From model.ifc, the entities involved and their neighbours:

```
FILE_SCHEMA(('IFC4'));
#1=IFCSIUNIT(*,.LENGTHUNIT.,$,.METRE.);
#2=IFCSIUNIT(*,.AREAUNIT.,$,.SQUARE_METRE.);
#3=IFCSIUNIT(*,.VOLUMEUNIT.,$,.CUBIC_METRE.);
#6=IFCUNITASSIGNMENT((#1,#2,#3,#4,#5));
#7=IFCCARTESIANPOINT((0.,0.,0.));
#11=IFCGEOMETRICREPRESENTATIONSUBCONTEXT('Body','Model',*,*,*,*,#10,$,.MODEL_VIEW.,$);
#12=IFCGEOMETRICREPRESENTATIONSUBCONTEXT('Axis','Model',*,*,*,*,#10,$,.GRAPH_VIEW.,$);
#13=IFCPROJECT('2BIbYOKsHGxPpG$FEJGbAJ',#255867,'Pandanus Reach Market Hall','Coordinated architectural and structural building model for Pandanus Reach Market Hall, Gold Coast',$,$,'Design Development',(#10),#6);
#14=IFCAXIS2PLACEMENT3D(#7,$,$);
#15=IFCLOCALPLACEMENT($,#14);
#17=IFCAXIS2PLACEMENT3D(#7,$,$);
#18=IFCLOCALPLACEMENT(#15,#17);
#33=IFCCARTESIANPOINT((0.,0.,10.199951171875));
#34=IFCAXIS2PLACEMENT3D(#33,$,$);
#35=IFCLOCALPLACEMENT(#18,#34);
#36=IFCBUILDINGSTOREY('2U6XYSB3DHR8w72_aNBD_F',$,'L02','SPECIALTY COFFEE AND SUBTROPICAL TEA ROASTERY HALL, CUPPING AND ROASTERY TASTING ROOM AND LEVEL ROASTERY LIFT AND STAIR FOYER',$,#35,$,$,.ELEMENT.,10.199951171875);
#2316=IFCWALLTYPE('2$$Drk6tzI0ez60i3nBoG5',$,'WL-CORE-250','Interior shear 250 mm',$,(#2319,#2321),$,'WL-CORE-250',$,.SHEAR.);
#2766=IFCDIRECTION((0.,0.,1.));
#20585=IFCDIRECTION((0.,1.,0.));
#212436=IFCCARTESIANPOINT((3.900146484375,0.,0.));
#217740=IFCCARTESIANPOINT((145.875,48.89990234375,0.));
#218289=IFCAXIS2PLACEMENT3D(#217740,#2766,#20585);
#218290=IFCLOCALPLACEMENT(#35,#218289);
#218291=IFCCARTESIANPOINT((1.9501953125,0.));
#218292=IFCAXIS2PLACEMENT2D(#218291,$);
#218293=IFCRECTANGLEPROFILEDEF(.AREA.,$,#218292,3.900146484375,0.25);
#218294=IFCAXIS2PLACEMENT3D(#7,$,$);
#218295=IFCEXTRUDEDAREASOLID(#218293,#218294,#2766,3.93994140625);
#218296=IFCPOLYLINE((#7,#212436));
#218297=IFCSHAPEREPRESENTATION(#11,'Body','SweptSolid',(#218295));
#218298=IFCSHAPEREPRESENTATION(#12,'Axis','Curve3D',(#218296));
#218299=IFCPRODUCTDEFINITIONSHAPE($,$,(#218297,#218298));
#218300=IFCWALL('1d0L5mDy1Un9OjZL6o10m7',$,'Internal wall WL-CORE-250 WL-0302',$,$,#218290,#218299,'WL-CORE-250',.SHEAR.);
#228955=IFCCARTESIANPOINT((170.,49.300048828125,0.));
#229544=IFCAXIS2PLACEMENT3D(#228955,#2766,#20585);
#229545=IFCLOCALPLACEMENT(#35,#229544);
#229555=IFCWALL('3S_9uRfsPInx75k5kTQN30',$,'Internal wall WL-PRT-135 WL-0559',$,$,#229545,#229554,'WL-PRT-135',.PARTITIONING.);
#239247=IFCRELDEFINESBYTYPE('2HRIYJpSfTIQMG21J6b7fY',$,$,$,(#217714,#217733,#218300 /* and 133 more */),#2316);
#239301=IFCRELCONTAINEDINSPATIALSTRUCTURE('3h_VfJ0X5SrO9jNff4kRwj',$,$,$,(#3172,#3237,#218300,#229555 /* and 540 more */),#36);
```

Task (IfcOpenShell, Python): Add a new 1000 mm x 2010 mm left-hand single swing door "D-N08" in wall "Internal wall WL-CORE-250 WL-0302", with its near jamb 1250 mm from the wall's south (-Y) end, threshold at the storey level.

```python
import numpy as np
import ifcopenshell
import ifcopenshell.api.feature
import ifcopenshell.api.geometry
import ifcopenshell.api.root
import ifcopenshell.api.spatial
import ifcopenshell.geom
import ifcopenshell.util.element
import ifcopenshell.util.placement
import ifcopenshell.util.representation
import ifcopenshell.util.shape
import ifcopenshell.util.unit

model = ifcopenshell.open("model.ifc")
unit_scale = ifcopenshell.util.unit.calculate_unit_scale(model)
settings = ifcopenshell.geom.settings()


def volume(element):
    """Net volume in cubic metres, openings subtracted."""
    shape = ifcopenshell.geom.create_shape(settings, element)
    return ifcopenshell.util.shape.get_volume(shape.geometry)


wall = model.by_guid("1d0L5mDy1Un9OjZL6o10m7")
storey = ifcopenshell.util.element.get_container(wall, ifc_class="IfcBuildingStorey")
context = ifcopenshell.util.representation.get_context(model, "Model", "Body", "MODEL_VIEW")
before = volume(wall)

width, height, from_end, sill = 1, 2.01, 1.25, 0.0  # metres

# The wall runs along its own X axis, and the end named is its -X end.
wall_shape = ifcopenshell.geom.create_shape(settings, wall)
x, y, z = ifcopenshell.util.shape.get_vertices(wall_shape.geometry).T
start = x.min() + from_end
face, thickness = float(y.min()), float(y.max() - y.min())
wall_matrix = ifcopenshell.util.placement.get_local_placement(wall.ObjectPlacement)
level = ifcopenshell.util.placement.get_local_placement(storey.ObjectPlacement)[2, 3]


def in_wall(x, y):
    """Placement at x, y metres in the wall's axes, at sill height."""
    matrix = wall_matrix.copy()
    matrix[:, 3] = wall_matrix @ np.array([x / unit_scale, y / unit_scale, 0.0, 1.0])
    matrix[2, 3] = level + sill / unit_scale
    return matrix


# Opening: a box that overshoots both wall faces by 50 mm.
opening = ifcopenshell.api.root.create_entity(model, ifc_class="IfcOpeningElement", predefined_type="OPENING")
box = ifcopenshell.api.geometry.add_wall_representation(
    model, context=context, length=width, height=height, thickness=thickness + 0.1
)
ifcopenshell.api.geometry.assign_representation(model, product=opening, representation=box)
ifcopenshell.api.geometry.edit_object_placement(model, product=opening, matrix=in_wall(start, face - 0.05), is_si=False)
ifcopenshell.api.feature.add_feature(model, feature=opening, element=wall)

door = ifcopenshell.api.root.create_entity(model, ifc_class="IfcDoor", name="D-N08", predefined_type="DOOR")
door.OverallWidth, door.OverallHeight = width / unit_scale, height / unit_scale
door.OperationType = "SINGLE_SWING_LEFT"
body = ifcopenshell.api.geometry.add_door_representation(
    model,
    context=context,
    overall_width=door.OverallWidth,
    overall_height=door.OverallHeight,
    operation_type="SINGLE_SWING_LEFT",
    lining_properties={"LiningDepth": thickness / unit_scale, "ThresholdDepth": thickness / unit_scale},
)
ifcopenshell.api.geometry.assign_representation(model, product=door, representation=body)
ifcopenshell.api.spatial.assign_container(model, products=[door], relating_structure=storey)
ifcopenshell.api.feature.add_filling(model, opening=opening, element=door)

# The lining spans the wall, so the door starts at the wall face.
ifcopenshell.api.geometry.edit_object_placement(model, product=door, matrix=in_wall(start, face), is_si=False)

after = volume(wall)

print(f"wall volume {before:.3f} -> {after:.3f} m3")

model.write("model_edited.ifc")
```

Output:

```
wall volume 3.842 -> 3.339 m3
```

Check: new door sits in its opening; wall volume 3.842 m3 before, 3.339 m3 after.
